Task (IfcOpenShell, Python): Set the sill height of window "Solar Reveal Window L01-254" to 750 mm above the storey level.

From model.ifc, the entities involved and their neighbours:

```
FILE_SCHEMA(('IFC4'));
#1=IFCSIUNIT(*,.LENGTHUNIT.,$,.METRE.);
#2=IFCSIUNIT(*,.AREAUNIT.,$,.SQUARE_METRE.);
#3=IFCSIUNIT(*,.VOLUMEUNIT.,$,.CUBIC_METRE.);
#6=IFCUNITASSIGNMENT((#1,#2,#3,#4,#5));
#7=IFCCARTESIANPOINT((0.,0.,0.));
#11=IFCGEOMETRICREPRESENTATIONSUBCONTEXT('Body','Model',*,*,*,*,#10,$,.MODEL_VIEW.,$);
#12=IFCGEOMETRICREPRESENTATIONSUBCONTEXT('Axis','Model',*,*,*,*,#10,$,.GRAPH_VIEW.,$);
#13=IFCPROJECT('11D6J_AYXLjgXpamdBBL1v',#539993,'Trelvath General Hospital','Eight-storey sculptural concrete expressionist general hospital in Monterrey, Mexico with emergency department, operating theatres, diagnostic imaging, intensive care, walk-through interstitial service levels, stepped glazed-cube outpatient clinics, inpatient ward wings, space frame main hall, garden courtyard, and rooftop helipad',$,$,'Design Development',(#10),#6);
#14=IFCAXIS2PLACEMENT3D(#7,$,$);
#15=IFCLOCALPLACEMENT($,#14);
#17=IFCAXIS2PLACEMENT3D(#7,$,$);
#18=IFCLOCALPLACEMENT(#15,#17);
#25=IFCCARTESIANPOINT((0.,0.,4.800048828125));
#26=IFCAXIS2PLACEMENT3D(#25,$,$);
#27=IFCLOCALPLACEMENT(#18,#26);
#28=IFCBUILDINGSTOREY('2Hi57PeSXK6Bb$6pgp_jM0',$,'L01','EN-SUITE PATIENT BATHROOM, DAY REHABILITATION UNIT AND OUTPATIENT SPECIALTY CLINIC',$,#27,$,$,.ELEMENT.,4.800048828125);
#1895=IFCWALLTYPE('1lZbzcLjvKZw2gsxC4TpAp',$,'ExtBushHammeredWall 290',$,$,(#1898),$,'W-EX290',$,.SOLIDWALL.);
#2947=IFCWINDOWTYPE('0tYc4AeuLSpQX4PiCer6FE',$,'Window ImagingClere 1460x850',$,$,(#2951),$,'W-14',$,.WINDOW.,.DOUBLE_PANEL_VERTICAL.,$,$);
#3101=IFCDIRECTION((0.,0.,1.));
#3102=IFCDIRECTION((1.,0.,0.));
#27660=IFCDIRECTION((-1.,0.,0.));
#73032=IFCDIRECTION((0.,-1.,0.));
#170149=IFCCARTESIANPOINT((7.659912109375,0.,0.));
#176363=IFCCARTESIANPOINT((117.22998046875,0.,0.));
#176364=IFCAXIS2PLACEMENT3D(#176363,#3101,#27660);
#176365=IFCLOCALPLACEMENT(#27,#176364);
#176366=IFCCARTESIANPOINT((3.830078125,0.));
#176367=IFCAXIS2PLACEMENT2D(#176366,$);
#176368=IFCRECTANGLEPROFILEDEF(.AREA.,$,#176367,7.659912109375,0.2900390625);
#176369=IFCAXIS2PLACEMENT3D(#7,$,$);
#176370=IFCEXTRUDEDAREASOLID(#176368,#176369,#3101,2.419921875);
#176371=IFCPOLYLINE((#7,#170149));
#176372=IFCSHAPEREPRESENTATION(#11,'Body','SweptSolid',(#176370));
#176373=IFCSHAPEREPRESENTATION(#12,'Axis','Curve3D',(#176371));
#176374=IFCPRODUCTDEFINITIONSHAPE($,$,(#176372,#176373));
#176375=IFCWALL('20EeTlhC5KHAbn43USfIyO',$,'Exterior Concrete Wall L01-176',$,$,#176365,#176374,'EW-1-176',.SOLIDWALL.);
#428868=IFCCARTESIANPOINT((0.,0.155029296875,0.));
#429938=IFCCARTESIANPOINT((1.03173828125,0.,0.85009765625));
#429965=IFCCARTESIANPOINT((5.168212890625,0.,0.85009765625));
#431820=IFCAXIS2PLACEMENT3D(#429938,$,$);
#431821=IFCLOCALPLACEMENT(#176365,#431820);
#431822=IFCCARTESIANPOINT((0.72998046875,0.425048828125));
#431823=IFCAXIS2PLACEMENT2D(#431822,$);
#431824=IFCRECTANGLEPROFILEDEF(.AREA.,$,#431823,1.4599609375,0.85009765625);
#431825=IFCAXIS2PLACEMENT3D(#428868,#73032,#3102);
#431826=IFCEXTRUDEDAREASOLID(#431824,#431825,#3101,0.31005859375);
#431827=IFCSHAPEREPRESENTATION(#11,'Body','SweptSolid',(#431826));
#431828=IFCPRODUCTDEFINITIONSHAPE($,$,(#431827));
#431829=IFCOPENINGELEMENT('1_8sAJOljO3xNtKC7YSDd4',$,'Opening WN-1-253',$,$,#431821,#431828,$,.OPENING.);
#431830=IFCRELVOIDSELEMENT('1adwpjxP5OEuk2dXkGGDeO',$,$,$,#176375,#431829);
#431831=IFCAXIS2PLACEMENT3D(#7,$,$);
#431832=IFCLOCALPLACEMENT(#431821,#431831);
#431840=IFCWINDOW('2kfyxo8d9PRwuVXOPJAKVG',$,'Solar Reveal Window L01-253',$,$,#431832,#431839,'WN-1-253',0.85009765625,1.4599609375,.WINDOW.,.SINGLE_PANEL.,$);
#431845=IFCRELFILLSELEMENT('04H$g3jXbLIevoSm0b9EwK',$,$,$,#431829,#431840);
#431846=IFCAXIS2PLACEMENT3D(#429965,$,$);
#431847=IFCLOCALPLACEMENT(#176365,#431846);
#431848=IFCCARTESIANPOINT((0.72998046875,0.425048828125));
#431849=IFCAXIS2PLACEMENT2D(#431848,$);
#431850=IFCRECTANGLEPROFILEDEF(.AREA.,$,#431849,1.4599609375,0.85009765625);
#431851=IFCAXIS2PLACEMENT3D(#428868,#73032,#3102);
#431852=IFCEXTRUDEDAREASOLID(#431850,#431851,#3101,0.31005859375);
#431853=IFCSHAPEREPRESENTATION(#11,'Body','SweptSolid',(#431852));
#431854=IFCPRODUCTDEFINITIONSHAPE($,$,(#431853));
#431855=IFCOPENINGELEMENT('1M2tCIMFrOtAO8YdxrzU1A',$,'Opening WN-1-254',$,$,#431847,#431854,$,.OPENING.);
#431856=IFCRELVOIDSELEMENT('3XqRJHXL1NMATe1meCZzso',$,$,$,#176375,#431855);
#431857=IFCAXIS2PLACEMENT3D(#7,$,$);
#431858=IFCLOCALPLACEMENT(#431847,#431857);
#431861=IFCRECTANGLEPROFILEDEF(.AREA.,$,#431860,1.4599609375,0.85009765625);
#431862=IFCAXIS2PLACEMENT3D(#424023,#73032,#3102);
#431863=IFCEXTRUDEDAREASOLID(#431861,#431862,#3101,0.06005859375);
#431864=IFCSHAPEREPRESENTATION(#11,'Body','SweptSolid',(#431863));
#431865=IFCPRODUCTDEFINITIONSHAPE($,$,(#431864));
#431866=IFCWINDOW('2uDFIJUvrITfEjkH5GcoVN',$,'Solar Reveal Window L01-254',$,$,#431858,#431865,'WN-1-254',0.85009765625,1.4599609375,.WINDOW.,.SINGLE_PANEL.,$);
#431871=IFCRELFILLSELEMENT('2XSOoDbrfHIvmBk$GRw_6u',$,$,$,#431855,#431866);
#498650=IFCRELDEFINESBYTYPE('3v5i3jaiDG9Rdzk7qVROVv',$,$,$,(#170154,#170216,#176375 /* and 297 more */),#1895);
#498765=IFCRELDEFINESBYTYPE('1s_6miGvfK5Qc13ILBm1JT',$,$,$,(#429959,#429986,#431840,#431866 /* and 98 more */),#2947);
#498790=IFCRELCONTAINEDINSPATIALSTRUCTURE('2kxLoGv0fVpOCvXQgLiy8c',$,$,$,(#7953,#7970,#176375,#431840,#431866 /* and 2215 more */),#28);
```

```python
import numpy as np
import ifcopenshell
import ifcopenshell.api.geometry
import ifcopenshell.geom
import ifcopenshell.util.element
import ifcopenshell.util.placement
import ifcopenshell.util.shape
import ifcopenshell.util.unit

model = ifcopenshell.open("model.ifc")
unit_scale = ifcopenshell.util.unit.calculate_unit_scale(model)

window = model.by_guid("2uDFIJUvrITfEjkH5GcoVN")
opening = window.FillsVoids[0].RelatingOpeningElement
storey = ifcopenshell.util.element.get_container(window, ifc_class="IfcBuildingStorey")
level = ifcopenshell.util.placement.get_local_placement(storey.ObjectPlacement)[2, 3]

# The opening's origin need not be at the sill, so measure its lowest point.
shape = ifcopenshell.geom.create_shape(ifcopenshell.geom.settings(), opening)
bottom = ifcopenshell.util.shape.get_shape_bottom_elevation(shape, shape.geometry) / unit_scale
dz = level + 0.75 - bottom

shift = np.array([0.0, 0.0, dz])
# The window is placed relative to its opening, so it follows when the opening moves.
matrix = ifcopenshell.util.placement.get_local_placement(opening.ObjectPlacement)
matrix[:3, 3] += shift
ifcopenshell.api.geometry.edit_object_placement(
    model, product=opening, matrix=matrix, is_si=False, should_transform_children=True
)

print(f"moved by {dz * unit_scale:+.3f} m")

model.write("model_rev.ifc")
```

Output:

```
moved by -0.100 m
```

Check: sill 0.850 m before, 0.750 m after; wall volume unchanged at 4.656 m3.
